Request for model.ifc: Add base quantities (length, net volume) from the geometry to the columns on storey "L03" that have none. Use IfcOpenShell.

First a look at what the model holds.

```python
import ifcopenshell
import ifcopenshell.util.element
import ifcopenshell.util.unit

model = ifcopenshell.open("model.ifc")
print(model.schema)
for unit_type in ("LENGTHUNIT", "AREAUNIT", "VOLUMEUNIT"):
    print(unit_type, ifcopenshell.util.unit.calculate_unit_scale(model, unit_type))
storey = next(s for s in model.by_type("IfcBuildingStorey") if s.Name == "L03")
columns = [e for e in ifcopenshell.util.element.get_decomposition(storey) if e.is_a("IfcColumn")]
for e in sorted(columns, key=lambda e: e.id()):
    print(e.id(), e.is_a(), e.Name, list(ifcopenshell.util.element.get_psets(e, qtos_only=True)), sep=" | ")
```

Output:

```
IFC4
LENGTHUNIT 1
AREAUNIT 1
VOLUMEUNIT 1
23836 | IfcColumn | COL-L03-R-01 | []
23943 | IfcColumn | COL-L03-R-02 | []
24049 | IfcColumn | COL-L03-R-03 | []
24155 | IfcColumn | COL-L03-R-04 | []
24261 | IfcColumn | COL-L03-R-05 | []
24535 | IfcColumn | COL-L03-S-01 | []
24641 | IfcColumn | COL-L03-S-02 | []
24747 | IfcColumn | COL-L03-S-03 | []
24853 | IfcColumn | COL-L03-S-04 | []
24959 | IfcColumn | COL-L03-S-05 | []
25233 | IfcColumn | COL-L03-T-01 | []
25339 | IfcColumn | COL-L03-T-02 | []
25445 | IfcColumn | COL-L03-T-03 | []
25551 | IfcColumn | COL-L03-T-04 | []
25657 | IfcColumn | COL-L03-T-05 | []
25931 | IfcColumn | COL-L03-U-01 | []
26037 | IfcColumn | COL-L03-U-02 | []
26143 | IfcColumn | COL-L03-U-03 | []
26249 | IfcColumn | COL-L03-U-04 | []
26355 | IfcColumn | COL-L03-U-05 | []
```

```python
import ifcopenshell
import ifcopenshell.api.pset
import ifcopenshell.geom
import ifcopenshell.util.element
import ifcopenshell.util.shape
import ifcopenshell.util.unit

model = ifcopenshell.open("model.ifc")
unit_scale = ifcopenshell.util.unit.calculate_unit_scale(model)
volume_scale = ifcopenshell.util.unit.calculate_unit_scale(model, "VOLUMEUNIT")
settings = ifcopenshell.geom.settings()

storey = next(s for s in model.by_type("IfcBuildingStorey") if s.Name == "L03")
columns = [e for e in ifcopenshell.util.element.get_decomposition(storey) if e.is_a("IfcColumn")]

for e in sorted(columns, key=lambda e: e.id()):
    if ifcopenshell.util.element.get_psets(e, qtos_only=True, should_inherit=False):
        continue
    # Geometry comes back in metres, in the element's own axes.
    shape = ifcopenshell.geom.create_shape(settings, e)
    values = {
        "Length": ifcopenshell.util.shape.get_z(shape.geometry) / unit_scale,
        "NetVolume": ifcopenshell.util.shape.get_volume(shape.geometry) / volume_scale,
    }
    qto = ifcopenshell.api.pset.add_qto(model, product=e, name="Qto_ColumnBaseQuantities")
    ifcopenshell.api.pset.edit_qto(model, qto=qto, properties=values)
    print(e.id(), {k: round(v, 3) for k, v in values.items()})

model.write("model_edited.ifc")
```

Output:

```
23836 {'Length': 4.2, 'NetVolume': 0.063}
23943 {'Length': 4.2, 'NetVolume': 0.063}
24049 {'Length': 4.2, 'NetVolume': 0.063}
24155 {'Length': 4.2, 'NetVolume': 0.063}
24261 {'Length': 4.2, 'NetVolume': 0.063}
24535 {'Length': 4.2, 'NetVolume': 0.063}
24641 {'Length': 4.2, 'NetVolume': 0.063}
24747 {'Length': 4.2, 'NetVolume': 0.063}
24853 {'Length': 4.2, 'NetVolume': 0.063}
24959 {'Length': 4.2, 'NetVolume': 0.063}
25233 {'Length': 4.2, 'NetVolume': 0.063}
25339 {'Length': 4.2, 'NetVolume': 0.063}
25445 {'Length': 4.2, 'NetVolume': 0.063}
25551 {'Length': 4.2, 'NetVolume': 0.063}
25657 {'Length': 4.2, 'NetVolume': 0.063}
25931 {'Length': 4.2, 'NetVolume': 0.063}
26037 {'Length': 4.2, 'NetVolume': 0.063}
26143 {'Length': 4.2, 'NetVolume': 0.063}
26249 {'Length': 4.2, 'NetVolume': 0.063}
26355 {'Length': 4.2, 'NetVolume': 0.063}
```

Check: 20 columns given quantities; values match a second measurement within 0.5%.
